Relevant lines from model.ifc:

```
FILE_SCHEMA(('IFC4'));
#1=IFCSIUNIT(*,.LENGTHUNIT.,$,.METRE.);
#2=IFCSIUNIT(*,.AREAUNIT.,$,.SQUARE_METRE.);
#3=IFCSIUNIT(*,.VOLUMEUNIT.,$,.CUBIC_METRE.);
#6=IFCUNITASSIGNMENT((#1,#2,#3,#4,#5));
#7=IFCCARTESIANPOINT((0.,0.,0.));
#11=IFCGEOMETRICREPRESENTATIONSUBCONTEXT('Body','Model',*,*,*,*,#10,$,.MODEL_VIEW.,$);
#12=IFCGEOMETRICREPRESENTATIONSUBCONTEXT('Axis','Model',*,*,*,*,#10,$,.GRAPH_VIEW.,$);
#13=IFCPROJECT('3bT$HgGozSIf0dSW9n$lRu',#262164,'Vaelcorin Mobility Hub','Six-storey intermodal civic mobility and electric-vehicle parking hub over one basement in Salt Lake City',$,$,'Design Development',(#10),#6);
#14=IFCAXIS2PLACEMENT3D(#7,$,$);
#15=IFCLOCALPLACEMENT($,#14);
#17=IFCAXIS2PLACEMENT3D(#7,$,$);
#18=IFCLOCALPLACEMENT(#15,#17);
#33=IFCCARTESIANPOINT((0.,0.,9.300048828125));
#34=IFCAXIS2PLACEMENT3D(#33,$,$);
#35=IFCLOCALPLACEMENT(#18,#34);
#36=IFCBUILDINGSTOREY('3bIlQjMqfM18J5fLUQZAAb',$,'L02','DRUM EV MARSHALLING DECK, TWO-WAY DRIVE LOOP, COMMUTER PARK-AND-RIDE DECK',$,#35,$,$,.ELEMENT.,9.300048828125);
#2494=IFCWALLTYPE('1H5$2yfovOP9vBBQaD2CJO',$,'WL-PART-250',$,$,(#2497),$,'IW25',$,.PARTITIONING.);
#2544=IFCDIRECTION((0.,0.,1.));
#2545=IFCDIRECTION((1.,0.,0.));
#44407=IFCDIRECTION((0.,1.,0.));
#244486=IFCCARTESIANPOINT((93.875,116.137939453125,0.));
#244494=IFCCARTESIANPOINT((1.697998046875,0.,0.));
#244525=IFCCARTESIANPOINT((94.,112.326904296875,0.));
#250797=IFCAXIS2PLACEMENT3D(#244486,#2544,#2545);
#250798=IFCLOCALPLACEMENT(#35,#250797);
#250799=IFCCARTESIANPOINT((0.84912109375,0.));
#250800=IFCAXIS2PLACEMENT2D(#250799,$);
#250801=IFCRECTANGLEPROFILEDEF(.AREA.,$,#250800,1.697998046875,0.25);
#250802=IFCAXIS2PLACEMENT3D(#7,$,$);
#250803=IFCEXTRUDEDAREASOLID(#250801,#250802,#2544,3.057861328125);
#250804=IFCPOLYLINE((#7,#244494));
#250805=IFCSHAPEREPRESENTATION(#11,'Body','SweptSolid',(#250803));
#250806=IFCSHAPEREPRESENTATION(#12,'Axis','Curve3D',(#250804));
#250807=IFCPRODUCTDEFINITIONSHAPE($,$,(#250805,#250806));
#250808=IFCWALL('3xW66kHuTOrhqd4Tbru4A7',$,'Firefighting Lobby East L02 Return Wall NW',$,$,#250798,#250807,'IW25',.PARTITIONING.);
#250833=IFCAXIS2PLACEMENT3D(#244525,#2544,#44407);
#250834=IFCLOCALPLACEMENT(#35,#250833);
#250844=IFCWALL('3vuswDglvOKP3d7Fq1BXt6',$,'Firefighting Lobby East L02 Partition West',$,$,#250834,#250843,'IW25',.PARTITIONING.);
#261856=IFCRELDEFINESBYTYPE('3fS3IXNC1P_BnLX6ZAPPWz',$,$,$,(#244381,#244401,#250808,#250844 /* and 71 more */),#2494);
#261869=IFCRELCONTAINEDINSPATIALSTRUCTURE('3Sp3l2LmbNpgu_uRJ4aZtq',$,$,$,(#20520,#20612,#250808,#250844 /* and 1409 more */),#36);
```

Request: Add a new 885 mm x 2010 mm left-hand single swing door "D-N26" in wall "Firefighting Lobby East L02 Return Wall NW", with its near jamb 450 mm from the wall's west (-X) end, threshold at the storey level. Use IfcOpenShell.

```python
import numpy as np
import ifcopenshell
import ifcopenshell.api.feature
import ifcopenshell.api.geometry
import ifcopenshell.api.root
import ifcopenshell.api.spatial
import ifcopenshell.geom
import ifcopenshell.util.element
import ifcopenshell.util.placement
import ifcopenshell.util.representation
import ifcopenshell.util.shape
import ifcopenshell.util.unit

model = ifcopenshell.open("model.ifc")
unit_scale = ifcopenshell.util.unit.calculate_unit_scale(model)
settings = ifcopenshell.geom.settings()


def volume(element):
    """Net volume in cubic metres, openings subtracted."""
    shape = ifcopenshell.geom.create_shape(settings, element)
    return ifcopenshell.util.shape.get_volume(shape.geometry)


wall = model.by_guid("3xW66kHuTOrhqd4Tbru4A7")
storey = ifcopenshell.util.element.get_container(wall, ifc_class="IfcBuildingStorey")
context = ifcopenshell.util.representation.get_context(model, "Model", "Body", "MODEL_VIEW")
before = volume(wall)

width, height, from_end, sill = 0.885, 2.01, 0.45, 0.0  # metres

# The wall runs along its own X axis, and the end named is its -X end.
wall_shape = ifcopenshell.geom.create_shape(settings, wall)
x, y, z = ifcopenshell.util.shape.get_vertices(wall_shape.geometry).T
start = x.min() + from_end
face, thickness = float(y.min()), float(y.max() - y.min())
wall_matrix = ifcopenshell.util.placement.get_local_placement(wall.ObjectPlacement)
level = ifcopenshell.util.placement.get_local_placement(storey.ObjectPlacement)[2, 3]


def in_wall(x, y):
    """Placement at x, y metres in the wall's axes, at sill height."""
    matrix = wall_matrix.copy()
    matrix[:, 3] = wall_matrix @ np.array([x / unit_scale, y / unit_scale, 0.0, 1.0])
    matrix[2, 3] = level + sill / unit_scale
    return matrix


# Opening: a box that overshoots both wall faces by 50 mm.
opening = ifcopenshell.api.root.create_entity(model, ifc_class="IfcOpeningElement", predefined_type="OPENING")
box = ifcopenshell.api.geometry.add_wall_representation(
    model, context=context, length=width, height=height, thickness=thickness + 0.1
)
ifcopenshell.api.geometry.assign_representation(model, product=opening, representation=box)
ifcopenshell.api.geometry.edit_object_placement(model, product=opening, matrix=in_wall(start, face - 0.05), is_si=False)
ifcopenshell.api.feature.add_feature(model, feature=opening, element=wall)

door = ifcopenshell.api.root.create_entity(model, ifc_class="IfcDoor", name="D-N26", predefined_type="DOOR")
door.OverallWidth, door.OverallHeight = width / unit_scale, height / unit_scale
door.OperationType = "SINGLE_SWING_LEFT"
body = ifcopenshell.api.geometry.add_door_representation(
    model,
    context=context,
    overall_width=door.OverallWidth,
    overall_height=door.OverallHeight,
    operation_type="SINGLE_SWING_LEFT",
    lining_properties={"LiningDepth": thickness / unit_scale, "ThresholdDepth": thickness / unit_scale},
)
ifcopenshell.api.geometry.assign_representation(model, product=door, representation=body)
ifcopenshell.api.spatial.assign_container(model, products=[door], relating_structure=storey)
ifcopenshell.api.feature.add_filling(model, opening=opening, element=door)

# The lining spans the wall, so the door starts at the wall face.
ifcopenshell.api.geometry.edit_object_placement(model, product=door, matrix=in_wall(start, face), is_si=False)

after = volume(wall)

print(f"wall volume {before:.3f} -> {after:.3f} m3")

model.write("model_updated.ifc")
```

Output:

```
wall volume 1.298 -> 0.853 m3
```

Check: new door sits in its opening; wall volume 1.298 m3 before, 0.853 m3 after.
